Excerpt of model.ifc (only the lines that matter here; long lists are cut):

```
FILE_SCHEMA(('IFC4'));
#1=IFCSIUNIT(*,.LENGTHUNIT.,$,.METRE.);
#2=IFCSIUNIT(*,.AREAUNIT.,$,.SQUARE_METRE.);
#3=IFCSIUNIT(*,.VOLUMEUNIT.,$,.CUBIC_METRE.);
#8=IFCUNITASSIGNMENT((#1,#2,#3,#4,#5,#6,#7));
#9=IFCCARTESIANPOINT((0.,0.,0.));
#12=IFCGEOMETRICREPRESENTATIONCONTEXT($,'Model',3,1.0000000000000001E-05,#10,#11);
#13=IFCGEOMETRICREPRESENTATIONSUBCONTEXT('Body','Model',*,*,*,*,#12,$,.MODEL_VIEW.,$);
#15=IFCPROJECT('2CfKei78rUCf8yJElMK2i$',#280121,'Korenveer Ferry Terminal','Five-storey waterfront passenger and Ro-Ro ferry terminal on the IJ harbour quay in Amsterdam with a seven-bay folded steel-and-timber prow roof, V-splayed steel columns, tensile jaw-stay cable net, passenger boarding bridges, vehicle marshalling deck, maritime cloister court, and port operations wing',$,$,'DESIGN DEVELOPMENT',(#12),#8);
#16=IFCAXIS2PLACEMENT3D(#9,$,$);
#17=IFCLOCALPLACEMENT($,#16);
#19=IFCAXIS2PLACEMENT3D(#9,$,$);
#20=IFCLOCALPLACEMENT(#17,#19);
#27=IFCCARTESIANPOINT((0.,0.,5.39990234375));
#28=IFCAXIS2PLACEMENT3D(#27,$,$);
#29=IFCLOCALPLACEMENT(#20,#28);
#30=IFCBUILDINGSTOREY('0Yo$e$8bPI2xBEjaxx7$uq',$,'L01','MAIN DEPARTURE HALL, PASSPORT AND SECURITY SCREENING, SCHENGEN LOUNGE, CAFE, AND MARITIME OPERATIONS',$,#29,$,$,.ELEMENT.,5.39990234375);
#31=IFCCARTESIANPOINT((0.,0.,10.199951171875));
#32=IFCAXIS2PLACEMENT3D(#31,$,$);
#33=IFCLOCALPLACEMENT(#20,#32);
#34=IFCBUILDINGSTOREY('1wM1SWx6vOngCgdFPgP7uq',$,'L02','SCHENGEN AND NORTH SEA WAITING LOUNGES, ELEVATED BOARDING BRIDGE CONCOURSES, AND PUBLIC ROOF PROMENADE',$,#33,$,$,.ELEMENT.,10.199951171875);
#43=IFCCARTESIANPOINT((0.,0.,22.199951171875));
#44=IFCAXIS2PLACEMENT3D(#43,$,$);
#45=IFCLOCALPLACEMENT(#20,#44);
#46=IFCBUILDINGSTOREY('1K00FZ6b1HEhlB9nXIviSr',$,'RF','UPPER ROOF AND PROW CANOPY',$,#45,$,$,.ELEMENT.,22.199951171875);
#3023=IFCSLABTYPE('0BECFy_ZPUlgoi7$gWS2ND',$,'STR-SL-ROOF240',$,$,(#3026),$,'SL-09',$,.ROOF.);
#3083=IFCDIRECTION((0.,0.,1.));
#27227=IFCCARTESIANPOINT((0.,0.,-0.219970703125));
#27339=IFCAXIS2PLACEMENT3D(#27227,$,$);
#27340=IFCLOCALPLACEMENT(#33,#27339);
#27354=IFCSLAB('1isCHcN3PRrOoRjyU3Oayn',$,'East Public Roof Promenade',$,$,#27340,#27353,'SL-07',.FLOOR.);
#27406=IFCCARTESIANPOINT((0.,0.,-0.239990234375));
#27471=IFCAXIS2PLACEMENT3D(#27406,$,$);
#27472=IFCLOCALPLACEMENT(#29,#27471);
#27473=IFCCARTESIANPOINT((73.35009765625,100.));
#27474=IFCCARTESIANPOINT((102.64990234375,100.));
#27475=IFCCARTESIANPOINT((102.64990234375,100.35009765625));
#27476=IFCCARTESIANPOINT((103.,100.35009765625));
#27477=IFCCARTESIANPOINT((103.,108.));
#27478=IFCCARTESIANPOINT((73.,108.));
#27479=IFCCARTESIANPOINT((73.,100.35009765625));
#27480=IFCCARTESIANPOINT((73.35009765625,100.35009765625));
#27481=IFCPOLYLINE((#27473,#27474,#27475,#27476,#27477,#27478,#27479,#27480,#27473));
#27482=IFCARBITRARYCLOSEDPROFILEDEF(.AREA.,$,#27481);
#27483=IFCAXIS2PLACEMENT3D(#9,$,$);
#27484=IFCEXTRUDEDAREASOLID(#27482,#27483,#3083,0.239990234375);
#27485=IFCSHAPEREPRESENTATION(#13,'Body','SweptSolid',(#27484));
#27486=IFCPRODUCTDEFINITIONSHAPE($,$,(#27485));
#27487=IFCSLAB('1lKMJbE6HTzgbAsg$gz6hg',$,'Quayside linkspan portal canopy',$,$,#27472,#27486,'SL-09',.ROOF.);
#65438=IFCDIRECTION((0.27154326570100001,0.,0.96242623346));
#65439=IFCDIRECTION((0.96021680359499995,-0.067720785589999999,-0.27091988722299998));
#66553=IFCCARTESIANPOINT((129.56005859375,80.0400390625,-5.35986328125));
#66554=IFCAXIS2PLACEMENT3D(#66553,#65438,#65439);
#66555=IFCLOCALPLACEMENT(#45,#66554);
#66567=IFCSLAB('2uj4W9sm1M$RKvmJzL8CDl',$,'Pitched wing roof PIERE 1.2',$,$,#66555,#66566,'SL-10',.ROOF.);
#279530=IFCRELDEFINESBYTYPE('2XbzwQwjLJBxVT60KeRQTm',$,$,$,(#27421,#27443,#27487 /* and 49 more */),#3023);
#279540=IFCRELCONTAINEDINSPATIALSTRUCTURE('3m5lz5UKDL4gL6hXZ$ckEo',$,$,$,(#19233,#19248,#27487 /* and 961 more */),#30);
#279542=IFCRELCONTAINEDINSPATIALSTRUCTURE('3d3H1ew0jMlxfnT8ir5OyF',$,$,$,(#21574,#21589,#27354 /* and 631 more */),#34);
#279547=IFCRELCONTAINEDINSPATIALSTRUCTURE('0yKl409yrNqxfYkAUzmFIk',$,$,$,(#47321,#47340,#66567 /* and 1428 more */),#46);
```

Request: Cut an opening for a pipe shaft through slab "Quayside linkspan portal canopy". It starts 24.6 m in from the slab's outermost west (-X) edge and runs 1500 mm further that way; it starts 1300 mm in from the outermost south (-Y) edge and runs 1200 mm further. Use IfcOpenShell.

```python
import numpy as np
import ifcopenshell
import ifcopenshell.api.feature
import ifcopenshell.api.geometry
import ifcopenshell.api.root
import ifcopenshell.geom
import ifcopenshell.util.placement
import ifcopenshell.util.representation
import ifcopenshell.util.shape
import ifcopenshell.util.unit

model = ifcopenshell.open("model.ifc")
unit_scale = ifcopenshell.util.unit.calculate_unit_scale(model)
settings = ifcopenshell.geom.settings()


def volume(element):
    """Net volume in cubic metres, openings subtracted."""
    shape = ifcopenshell.geom.create_shape(settings, element)
    return ifcopenshell.util.shape.get_volume(shape.geometry)


slab = model.by_guid("1lKMJbE6HTzgbAsg$gz6hg")
before = volume(slab)

# Extent in the slab's own axes, in metres. The edges named are its -X and -Y sides.
slab_shape = ifcopenshell.geom.create_shape(settings, slab)
vertices = ifcopenshell.util.shape.get_vertices(slab_shape.geometry)
x_min, y_min, bottom = vertices.min(axis=0)
top = vertices[:, 2].max()

opening = ifcopenshell.api.root.create_entity(model, ifc_class="IfcOpeningElement", name="Pipe shaft opening", predefined_type="OPENING")
context = ifcopenshell.util.representation.get_context(model, "Model", "Body", "MODEL_VIEW")
width, depth = 1.5, 1.2
outline = [(0.0, 0.0), (width, 0.0), (width, depth), (0.0, depth), (0.0, 0.0)]
# Overshoot both faces by 50 mm so the cut is clean.
shape = ifcopenshell.api.geometry.add_slab_representation(
    model, context=context, depth=top - bottom + 0.1, polyline=outline
)
ifcopenshell.api.geometry.assign_representation(model, product=opening, representation=shape)

matrix = ifcopenshell.util.placement.get_local_placement(slab.ObjectPlacement)
matrix[:, 3] = matrix @ np.append(np.array([x_min + 24.6, y_min + 1.3, bottom - 0.05]) / unit_scale, 1.0)
ifcopenshell.api.geometry.edit_object_placement(model, product=opening, matrix=matrix, is_si=False)
ifcopenshell.api.feature.add_feature(model, feature=opening, element=slab)

after = volume(slab)

print(f"slab volume {before:.3f} -> {after:.3f} m3")

model.write("model-out.ifc")
```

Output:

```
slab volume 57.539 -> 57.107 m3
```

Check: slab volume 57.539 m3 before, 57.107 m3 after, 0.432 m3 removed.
